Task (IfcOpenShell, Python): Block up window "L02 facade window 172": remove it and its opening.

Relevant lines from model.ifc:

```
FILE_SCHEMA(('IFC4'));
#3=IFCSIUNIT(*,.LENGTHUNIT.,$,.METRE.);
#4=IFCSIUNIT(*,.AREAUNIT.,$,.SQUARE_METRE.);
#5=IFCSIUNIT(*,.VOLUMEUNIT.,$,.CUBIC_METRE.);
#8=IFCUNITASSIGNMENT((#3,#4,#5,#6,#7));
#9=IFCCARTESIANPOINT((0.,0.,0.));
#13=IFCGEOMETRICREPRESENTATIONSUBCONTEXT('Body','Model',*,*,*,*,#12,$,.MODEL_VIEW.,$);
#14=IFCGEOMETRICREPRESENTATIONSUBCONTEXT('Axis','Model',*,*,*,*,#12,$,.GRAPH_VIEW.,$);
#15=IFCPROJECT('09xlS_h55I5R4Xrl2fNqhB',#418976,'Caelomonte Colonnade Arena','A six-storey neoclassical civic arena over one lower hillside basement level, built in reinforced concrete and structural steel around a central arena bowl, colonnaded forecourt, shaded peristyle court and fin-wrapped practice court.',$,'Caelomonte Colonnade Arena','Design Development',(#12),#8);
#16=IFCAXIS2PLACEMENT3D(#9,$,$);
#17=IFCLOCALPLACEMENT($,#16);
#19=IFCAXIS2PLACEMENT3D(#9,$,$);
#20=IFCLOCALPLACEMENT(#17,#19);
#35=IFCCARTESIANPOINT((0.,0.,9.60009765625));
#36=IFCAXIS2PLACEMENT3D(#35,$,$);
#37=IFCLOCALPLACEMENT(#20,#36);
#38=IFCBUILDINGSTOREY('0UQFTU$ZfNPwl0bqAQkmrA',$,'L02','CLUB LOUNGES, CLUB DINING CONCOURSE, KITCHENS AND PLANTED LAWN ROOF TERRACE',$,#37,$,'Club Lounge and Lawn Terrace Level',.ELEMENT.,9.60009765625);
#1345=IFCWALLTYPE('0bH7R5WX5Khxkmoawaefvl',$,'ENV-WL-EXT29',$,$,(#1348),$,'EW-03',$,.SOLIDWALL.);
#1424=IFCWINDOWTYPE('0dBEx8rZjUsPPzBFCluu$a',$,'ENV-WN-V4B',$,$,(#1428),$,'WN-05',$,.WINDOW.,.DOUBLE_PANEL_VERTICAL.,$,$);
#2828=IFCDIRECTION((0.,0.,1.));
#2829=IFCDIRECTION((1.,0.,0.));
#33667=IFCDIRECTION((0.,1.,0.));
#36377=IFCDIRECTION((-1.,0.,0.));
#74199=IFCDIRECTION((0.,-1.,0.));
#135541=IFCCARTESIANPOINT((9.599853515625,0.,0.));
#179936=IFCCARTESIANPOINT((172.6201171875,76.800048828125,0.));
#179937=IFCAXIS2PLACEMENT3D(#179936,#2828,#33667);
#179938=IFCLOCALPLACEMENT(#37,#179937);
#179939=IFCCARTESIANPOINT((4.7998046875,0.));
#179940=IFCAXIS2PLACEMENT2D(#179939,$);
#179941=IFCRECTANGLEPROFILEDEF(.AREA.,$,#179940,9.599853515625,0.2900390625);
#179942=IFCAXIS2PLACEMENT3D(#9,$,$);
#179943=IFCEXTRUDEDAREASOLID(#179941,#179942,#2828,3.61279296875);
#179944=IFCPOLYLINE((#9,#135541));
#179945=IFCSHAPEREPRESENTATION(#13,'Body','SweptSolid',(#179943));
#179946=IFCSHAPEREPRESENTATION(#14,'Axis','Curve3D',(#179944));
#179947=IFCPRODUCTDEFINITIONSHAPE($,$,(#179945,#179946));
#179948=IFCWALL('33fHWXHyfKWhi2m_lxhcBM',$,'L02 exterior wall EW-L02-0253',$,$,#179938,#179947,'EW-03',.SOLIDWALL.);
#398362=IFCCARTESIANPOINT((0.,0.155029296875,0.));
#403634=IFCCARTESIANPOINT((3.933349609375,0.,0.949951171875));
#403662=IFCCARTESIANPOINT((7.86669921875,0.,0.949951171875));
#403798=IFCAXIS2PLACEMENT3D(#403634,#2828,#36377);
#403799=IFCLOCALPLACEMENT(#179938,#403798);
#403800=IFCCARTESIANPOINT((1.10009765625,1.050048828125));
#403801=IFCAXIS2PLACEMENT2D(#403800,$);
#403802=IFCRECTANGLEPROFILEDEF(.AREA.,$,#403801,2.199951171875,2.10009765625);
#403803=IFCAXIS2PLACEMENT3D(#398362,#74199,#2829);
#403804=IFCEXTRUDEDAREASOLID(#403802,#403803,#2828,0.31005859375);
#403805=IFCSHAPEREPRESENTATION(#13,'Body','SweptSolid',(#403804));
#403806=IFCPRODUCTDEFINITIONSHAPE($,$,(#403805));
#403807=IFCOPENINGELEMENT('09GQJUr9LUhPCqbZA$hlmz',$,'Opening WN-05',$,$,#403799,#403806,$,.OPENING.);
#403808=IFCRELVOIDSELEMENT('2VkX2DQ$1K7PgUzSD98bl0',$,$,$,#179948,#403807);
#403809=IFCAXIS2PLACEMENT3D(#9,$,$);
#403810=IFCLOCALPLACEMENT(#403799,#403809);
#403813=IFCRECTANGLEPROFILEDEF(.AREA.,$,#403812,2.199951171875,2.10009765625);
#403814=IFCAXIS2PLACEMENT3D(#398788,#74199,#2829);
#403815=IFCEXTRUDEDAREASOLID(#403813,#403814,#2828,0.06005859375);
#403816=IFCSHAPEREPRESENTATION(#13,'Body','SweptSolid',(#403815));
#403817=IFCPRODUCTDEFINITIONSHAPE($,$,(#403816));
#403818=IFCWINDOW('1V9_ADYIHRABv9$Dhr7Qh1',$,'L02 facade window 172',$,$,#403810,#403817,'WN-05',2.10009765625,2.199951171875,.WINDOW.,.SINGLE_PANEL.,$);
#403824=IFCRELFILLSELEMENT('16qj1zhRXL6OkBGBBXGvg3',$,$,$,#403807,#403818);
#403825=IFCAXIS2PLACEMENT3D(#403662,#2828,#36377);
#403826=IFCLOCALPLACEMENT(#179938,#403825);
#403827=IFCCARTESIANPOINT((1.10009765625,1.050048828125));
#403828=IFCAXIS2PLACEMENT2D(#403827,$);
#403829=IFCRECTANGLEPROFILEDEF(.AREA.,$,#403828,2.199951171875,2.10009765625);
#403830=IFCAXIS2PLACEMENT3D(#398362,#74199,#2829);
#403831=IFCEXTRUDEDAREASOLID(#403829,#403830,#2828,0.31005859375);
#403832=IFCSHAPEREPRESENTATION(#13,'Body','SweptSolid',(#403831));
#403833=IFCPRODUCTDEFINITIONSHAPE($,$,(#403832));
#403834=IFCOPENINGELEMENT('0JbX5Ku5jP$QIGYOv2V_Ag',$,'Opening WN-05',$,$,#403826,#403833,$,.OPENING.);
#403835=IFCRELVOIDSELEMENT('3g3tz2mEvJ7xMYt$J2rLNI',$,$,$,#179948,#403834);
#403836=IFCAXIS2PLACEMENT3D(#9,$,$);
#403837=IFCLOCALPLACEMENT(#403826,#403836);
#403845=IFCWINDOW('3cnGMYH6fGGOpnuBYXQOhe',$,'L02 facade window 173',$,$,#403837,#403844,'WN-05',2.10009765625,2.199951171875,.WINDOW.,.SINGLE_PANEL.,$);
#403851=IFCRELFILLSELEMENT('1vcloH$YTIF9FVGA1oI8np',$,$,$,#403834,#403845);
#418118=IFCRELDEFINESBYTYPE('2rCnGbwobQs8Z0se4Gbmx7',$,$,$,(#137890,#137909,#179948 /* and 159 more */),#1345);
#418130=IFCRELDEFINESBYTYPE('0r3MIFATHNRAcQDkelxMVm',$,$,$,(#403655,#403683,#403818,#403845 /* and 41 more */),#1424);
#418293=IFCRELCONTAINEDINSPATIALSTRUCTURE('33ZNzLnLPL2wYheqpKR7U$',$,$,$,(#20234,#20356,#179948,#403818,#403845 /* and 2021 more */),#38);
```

```python
import ifcopenshell
import ifcopenshell.api.feature
import ifcopenshell.api.root
import ifcopenshell.geom
import ifcopenshell.util.shape

model = ifcopenshell.open("model.ifc")
settings = ifcopenshell.geom.settings()


def volume(element):
    """Net volume in cubic metres, openings subtracted."""
    shape = ifcopenshell.geom.create_shape(settings, element)
    return ifcopenshell.util.shape.get_volume(shape.geometry)


window = model.by_guid("1V9_ADYIHRABv9$Dhr7Qh1")
opening = window.FillsVoids[0].RelatingOpeningElement
wall = opening.VoidsElements[0].RelatingBuildingElement
before = volume(wall)

ifcopenshell.api.root.remove_product(model, product=window)
ifcopenshell.api.feature.remove_feature(model, feature=opening)

after = volume(wall)

print(f"wall volume {before:.3f} -> {after:.3f} m3")

model.write("model_v2.ifc")
```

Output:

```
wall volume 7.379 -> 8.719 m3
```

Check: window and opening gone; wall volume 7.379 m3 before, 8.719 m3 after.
